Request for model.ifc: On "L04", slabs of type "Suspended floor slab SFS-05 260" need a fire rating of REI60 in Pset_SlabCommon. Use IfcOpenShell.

First a look at what the model holds.

```python
import ifcopenshell
import ifcopenshell.util.element

model = ifcopenshell.open("model.ifc")
print(model.schema)
storey = next(s for s in model.by_type("IfcBuildingStorey") if s.Name == "L04")
slabs = [e for e in ifcopenshell.util.element.get_decomposition(storey) if e.is_a("IfcSlab")]
seen = {}
for e in slabs:
    element_type = ifcopenshell.util.element.get_type(e)
    key = (element_type.Name if element_type != e and element_type else None, ifcopenshell.util.element.get_pset(e, "Pset_SlabCommon", "FireRating"))
    seen[key] = seen.get(key, 0) + 1
for (name, value), count in sorted(seen.items(), key=str):
    print(count, "x", name, "|", value)
```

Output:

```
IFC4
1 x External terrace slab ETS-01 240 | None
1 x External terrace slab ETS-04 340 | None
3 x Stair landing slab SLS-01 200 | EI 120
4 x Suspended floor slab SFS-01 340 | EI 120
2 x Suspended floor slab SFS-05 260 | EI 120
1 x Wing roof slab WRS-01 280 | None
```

```python
import ifcopenshell
import ifcopenshell.api.pset
import ifcopenshell.util.element

model = ifcopenshell.open("model.ifc")

storey = next(s for s in model.by_type("IfcBuildingStorey") if s.Name == "L04")
slabs = [e for e in ifcopenshell.util.element.get_decomposition(storey) if e.is_a("IfcSlab")]

count = 0
for e in slabs:
    element_type = ifcopenshell.util.element.get_type(e)
    if element_type in (None, e) or element_type.Name != "Suspended floor slab SFS-05 260":
        continue
    # add_pset returns the element's existing set when there is one.
    pset = ifcopenshell.api.pset.add_pset(model, product=e, name="Pset_SlabCommon")
    ifcopenshell.api.pset.edit_pset(model, pset=pset, properties={"FireRating": "REI60"})
    count += 1

print(count, "slabs updated")

model.write("model_edited.ifc")
```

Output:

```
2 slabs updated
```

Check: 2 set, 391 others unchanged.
